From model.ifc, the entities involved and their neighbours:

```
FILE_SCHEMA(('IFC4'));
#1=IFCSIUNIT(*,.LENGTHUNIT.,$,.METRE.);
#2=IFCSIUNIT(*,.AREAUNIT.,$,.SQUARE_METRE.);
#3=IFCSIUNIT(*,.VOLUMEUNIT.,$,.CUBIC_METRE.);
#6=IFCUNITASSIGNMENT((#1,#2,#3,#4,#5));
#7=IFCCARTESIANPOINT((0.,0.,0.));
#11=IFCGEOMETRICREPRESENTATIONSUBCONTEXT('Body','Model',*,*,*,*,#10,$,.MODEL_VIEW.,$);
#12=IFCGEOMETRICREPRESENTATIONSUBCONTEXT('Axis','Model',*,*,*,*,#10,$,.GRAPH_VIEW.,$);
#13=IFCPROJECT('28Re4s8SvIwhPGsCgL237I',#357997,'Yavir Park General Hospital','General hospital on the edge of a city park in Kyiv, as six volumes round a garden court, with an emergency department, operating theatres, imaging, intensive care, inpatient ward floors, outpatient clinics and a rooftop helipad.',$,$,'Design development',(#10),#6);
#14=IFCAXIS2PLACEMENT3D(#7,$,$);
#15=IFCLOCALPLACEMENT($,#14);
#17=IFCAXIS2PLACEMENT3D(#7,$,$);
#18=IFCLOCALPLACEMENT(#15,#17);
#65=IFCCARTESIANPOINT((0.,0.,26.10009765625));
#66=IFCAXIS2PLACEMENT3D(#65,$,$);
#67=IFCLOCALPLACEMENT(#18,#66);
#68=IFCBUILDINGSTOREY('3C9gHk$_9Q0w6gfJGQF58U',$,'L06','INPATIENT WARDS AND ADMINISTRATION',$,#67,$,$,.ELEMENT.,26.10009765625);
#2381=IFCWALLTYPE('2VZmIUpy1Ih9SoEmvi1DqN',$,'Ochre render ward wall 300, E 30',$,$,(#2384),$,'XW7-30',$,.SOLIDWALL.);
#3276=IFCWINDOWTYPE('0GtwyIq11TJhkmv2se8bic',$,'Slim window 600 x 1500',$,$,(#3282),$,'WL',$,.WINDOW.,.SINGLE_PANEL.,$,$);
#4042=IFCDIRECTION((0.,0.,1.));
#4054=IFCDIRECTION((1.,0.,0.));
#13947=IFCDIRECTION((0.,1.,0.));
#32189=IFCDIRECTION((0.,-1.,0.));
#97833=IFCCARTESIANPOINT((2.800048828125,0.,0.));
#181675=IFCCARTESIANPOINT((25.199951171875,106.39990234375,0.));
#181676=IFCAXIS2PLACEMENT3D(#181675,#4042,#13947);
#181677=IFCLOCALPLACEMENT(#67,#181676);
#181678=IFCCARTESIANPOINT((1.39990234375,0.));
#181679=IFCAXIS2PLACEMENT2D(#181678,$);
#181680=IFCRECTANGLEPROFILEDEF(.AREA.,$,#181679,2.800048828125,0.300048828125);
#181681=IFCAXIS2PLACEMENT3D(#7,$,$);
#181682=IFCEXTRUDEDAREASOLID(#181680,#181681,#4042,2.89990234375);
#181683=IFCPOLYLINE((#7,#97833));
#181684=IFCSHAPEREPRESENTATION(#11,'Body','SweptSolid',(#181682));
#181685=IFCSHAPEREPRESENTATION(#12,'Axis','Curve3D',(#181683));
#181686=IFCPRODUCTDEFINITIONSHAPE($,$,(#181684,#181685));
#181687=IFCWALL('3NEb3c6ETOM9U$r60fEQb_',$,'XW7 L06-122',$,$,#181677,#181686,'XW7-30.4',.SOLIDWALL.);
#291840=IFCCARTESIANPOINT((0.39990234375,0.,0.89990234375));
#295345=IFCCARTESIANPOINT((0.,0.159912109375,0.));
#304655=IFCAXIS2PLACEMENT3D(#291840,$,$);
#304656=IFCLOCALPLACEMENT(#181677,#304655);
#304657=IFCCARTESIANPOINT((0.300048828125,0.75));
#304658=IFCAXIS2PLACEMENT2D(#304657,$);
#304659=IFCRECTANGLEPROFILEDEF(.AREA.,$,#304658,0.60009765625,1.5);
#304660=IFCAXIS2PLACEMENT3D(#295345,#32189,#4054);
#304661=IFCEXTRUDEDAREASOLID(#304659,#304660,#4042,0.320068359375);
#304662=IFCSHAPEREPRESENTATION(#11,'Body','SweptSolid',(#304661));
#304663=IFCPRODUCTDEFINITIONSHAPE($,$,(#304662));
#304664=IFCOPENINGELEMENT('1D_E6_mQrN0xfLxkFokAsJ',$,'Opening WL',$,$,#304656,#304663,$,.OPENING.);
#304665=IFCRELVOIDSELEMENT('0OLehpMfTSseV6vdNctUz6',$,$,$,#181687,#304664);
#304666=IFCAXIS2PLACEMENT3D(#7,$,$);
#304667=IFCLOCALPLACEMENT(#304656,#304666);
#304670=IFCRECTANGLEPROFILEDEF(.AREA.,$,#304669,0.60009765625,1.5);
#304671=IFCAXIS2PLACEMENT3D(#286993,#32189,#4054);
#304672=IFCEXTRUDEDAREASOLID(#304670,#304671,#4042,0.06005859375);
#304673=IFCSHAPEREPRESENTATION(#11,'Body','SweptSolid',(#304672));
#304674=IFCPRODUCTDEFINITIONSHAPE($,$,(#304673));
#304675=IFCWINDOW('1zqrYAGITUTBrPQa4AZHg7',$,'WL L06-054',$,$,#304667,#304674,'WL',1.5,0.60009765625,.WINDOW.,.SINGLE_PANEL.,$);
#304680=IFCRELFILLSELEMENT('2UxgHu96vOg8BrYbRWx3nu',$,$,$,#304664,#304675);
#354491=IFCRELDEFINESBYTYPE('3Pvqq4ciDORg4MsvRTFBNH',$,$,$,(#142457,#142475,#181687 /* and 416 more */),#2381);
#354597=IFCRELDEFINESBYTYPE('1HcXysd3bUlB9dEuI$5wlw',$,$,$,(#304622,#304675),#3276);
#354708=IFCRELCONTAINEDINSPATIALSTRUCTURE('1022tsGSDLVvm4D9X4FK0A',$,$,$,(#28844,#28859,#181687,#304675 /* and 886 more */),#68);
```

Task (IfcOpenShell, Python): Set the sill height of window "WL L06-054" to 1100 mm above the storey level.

```python
import numpy as np
import ifcopenshell
import ifcopenshell.api.geometry
import ifcopenshell.geom
import ifcopenshell.util.element
import ifcopenshell.util.placement
import ifcopenshell.util.shape
import ifcopenshell.util.unit

model = ifcopenshell.open("model.ifc")
unit_scale = ifcopenshell.util.unit.calculate_unit_scale(model)

window = model.by_id(304675)
opening = window.FillsVoids[0].RelatingOpeningElement
storey = ifcopenshell.util.element.get_container(window, ifc_class="IfcBuildingStorey")
level = ifcopenshell.util.placement.get_local_placement(storey.ObjectPlacement)[2, 3]

# The opening's origin need not be at the sill, so measure its lowest point.
shape = ifcopenshell.geom.create_shape(ifcopenshell.geom.settings(), opening)
bottom = ifcopenshell.util.shape.get_shape_bottom_elevation(shape, shape.geometry) / unit_scale
dz = level + 1.1 - bottom

shift = np.array([0.0, 0.0, dz])
# The window is placed relative to its opening, so it follows when the opening moves.
matrix = ifcopenshell.util.placement.get_local_placement(opening.ObjectPlacement)
matrix[:3, 3] += shift
ifcopenshell.api.geometry.edit_object_placement(
    model, product=opening, matrix=matrix, is_si=False, should_transform_children=True
)

print(f"moved by {dz * unit_scale:+.3f} m")

model.write("model_v2.ifc")
```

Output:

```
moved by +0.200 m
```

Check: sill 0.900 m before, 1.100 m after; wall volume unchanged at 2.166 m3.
